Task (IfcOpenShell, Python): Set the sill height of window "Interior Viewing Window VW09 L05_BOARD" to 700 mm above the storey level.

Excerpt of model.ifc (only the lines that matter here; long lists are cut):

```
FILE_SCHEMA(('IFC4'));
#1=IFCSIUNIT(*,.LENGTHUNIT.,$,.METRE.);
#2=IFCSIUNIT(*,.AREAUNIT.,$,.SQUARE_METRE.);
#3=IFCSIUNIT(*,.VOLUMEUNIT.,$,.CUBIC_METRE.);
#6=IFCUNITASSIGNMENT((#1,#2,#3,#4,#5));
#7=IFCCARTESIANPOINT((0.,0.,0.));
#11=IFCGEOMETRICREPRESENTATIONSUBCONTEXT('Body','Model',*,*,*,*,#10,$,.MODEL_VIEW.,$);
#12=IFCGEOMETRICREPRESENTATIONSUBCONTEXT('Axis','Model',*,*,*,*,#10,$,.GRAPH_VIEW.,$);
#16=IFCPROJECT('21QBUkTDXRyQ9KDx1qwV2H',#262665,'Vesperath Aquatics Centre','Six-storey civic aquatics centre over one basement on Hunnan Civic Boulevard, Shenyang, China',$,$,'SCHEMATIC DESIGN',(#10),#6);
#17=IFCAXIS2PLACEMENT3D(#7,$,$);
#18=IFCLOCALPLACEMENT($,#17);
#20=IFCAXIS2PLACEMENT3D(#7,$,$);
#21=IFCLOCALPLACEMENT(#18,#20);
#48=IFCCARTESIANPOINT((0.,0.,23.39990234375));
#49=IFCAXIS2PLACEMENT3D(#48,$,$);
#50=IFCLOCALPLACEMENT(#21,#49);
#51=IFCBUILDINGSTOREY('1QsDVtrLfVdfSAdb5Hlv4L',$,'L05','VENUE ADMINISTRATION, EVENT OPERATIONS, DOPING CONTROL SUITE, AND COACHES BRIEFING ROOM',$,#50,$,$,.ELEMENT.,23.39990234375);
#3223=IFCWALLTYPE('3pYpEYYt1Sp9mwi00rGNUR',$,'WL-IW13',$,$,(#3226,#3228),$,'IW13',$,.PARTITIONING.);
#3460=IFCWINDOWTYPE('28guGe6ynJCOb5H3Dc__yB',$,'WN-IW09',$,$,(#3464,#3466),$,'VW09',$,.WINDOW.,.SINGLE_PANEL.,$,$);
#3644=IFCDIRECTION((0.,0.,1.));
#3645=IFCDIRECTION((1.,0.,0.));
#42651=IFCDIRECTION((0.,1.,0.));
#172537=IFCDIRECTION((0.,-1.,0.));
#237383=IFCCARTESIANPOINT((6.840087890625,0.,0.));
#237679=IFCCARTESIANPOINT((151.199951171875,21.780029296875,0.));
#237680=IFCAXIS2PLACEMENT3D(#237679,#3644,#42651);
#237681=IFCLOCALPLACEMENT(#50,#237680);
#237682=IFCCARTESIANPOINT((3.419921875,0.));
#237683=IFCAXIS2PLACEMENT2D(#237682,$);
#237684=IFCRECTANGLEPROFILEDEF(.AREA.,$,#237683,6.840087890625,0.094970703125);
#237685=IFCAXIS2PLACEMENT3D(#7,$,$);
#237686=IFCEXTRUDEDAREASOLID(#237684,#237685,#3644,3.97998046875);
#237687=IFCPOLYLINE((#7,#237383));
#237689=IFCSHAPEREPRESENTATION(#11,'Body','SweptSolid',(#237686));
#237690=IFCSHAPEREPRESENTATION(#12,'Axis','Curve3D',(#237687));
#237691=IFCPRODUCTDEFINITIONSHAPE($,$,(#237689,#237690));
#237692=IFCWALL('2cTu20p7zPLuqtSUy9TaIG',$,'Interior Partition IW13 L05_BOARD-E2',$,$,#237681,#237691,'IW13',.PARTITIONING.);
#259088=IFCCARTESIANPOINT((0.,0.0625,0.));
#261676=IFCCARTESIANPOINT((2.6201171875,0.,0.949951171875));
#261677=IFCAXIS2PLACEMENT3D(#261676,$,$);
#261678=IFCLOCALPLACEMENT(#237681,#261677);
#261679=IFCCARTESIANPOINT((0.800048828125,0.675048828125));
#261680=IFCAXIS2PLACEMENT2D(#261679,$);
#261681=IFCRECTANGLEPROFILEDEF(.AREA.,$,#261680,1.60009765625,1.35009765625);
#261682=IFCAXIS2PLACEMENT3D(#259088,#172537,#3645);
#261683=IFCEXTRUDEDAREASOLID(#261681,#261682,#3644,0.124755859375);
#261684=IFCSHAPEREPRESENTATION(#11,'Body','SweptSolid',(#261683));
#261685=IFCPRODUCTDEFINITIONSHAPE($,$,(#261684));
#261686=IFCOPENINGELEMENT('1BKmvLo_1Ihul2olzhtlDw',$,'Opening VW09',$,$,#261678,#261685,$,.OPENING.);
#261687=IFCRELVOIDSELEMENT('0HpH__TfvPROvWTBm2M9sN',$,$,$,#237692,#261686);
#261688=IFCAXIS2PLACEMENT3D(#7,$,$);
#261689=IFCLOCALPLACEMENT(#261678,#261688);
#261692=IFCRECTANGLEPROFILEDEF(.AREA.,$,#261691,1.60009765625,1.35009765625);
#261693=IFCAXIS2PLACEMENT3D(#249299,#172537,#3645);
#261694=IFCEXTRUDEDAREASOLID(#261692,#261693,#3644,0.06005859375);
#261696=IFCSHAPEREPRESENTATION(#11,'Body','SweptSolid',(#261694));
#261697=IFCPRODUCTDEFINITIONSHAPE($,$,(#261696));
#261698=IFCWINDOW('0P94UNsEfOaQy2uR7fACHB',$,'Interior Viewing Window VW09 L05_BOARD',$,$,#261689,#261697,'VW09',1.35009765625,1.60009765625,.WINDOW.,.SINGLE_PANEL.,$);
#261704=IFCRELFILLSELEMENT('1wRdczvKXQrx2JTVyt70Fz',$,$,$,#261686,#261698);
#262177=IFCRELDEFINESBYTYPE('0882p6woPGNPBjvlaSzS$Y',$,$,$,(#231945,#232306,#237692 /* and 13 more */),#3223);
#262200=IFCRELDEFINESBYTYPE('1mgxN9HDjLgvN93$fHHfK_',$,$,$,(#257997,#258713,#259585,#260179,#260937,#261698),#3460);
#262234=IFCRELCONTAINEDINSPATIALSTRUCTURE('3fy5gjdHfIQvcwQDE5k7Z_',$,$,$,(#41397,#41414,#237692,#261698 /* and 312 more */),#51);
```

```python
import numpy as np
import ifcopenshell
import ifcopenshell.api.geometry
import ifcopenshell.geom
import ifcopenshell.util.element
import ifcopenshell.util.placement
import ifcopenshell.util.shape
import ifcopenshell.util.unit

model = ifcopenshell.open("model.ifc")
unit_scale = ifcopenshell.util.unit.calculate_unit_scale(model)

window = model.by_guid("0P94UNsEfOaQy2uR7fACHB")
opening = window.FillsVoids[0].RelatingOpeningElement
storey = ifcopenshell.util.element.get_container(window, ifc_class="IfcBuildingStorey")
level = ifcopenshell.util.placement.get_local_placement(storey.ObjectPlacement)[2, 3]

# The opening's origin need not be at the sill, so measure its lowest point.
shape = ifcopenshell.geom.create_shape(ifcopenshell.geom.settings(), opening)
bottom = ifcopenshell.util.shape.get_shape_bottom_elevation(shape, shape.geometry) / unit_scale
dz = level + 0.7 / unit_scale - bottom

shift = np.array([0.0, 0.0, dz])
# The window is placed relative to its opening, so it follows when the opening moves.
matrix = ifcopenshell.util.placement.get_local_placement(opening.ObjectPlacement)
matrix[:3, 3] += shift
ifcopenshell.api.geometry.edit_object_placement(
    model, product=opening, matrix=matrix, is_si=False, should_transform_children=True
)

print(f"moved by {dz * unit_scale:+.3f} m")

model.write("model_edited.ifc")
```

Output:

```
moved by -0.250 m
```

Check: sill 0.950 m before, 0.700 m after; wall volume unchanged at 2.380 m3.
